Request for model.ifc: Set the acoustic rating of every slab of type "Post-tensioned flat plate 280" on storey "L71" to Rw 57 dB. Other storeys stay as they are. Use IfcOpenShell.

First a look at what the model holds.

```python
import ifcopenshell
import ifcopenshell.util.element

model = ifcopenshell.open("model.ifc")
print(model.schema)
storey = next(s for s in model.by_type("IfcBuildingStorey") if s.Name == "L71")
slabs = [e for e in ifcopenshell.util.element.get_decomposition(storey) if e.is_a("IfcSlab")]
seen = {}
for e in slabs:
    element_type = ifcopenshell.util.element.get_type(e)
    key = (element_type.Name if element_type != e and element_type else None, ifcopenshell.util.element.get_pset(e, "Pset_SlabCommon", "AcousticRating"))
    seen[key] = seen.get(key, 0) + 1
for (name, value), count in sorted(seen.items(), key=str):
    print(count, "x", name, "|", value)
```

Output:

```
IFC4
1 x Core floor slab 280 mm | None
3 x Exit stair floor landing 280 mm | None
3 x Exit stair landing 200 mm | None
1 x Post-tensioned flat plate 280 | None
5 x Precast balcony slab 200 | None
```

```python
import ifcopenshell
import ifcopenshell.api.pset
import ifcopenshell.util.element

model = ifcopenshell.open("model.ifc")

storey = next(s for s in model.by_type("IfcBuildingStorey") if s.Name == "L71")
slabs = [e for e in ifcopenshell.util.element.get_decomposition(storey) if e.is_a("IfcSlab")]

count = 0
for e in slabs:
    element_type = ifcopenshell.util.element.get_type(e)
    if element_type in (None, e) or element_type.Name != "Post-tensioned flat plate 280":
        continue
    found = ifcopenshell.util.element.get_pset(e, "Pset_SlabCommon", should_inherit=False)
    if found:
        pset = model.by_id(found["id"])
        if len(ifcopenshell.util.element.get_elements_by_pset(pset)) > 1:
            pset = ifcopenshell.api.pset.unshare_pset(model, products=[e], pset=pset)[0]
    else:
        pset = ifcopenshell.api.pset.add_pset(model, product=e, name="Pset_SlabCommon")
    ifcopenshell.api.pset.edit_pset(model, pset=pset, properties={"AcousticRating": "Rw 57 dB"})
    count += 1

print(count, "slabs updated")

model.write("model_v2.ifc")
```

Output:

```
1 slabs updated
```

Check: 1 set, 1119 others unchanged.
